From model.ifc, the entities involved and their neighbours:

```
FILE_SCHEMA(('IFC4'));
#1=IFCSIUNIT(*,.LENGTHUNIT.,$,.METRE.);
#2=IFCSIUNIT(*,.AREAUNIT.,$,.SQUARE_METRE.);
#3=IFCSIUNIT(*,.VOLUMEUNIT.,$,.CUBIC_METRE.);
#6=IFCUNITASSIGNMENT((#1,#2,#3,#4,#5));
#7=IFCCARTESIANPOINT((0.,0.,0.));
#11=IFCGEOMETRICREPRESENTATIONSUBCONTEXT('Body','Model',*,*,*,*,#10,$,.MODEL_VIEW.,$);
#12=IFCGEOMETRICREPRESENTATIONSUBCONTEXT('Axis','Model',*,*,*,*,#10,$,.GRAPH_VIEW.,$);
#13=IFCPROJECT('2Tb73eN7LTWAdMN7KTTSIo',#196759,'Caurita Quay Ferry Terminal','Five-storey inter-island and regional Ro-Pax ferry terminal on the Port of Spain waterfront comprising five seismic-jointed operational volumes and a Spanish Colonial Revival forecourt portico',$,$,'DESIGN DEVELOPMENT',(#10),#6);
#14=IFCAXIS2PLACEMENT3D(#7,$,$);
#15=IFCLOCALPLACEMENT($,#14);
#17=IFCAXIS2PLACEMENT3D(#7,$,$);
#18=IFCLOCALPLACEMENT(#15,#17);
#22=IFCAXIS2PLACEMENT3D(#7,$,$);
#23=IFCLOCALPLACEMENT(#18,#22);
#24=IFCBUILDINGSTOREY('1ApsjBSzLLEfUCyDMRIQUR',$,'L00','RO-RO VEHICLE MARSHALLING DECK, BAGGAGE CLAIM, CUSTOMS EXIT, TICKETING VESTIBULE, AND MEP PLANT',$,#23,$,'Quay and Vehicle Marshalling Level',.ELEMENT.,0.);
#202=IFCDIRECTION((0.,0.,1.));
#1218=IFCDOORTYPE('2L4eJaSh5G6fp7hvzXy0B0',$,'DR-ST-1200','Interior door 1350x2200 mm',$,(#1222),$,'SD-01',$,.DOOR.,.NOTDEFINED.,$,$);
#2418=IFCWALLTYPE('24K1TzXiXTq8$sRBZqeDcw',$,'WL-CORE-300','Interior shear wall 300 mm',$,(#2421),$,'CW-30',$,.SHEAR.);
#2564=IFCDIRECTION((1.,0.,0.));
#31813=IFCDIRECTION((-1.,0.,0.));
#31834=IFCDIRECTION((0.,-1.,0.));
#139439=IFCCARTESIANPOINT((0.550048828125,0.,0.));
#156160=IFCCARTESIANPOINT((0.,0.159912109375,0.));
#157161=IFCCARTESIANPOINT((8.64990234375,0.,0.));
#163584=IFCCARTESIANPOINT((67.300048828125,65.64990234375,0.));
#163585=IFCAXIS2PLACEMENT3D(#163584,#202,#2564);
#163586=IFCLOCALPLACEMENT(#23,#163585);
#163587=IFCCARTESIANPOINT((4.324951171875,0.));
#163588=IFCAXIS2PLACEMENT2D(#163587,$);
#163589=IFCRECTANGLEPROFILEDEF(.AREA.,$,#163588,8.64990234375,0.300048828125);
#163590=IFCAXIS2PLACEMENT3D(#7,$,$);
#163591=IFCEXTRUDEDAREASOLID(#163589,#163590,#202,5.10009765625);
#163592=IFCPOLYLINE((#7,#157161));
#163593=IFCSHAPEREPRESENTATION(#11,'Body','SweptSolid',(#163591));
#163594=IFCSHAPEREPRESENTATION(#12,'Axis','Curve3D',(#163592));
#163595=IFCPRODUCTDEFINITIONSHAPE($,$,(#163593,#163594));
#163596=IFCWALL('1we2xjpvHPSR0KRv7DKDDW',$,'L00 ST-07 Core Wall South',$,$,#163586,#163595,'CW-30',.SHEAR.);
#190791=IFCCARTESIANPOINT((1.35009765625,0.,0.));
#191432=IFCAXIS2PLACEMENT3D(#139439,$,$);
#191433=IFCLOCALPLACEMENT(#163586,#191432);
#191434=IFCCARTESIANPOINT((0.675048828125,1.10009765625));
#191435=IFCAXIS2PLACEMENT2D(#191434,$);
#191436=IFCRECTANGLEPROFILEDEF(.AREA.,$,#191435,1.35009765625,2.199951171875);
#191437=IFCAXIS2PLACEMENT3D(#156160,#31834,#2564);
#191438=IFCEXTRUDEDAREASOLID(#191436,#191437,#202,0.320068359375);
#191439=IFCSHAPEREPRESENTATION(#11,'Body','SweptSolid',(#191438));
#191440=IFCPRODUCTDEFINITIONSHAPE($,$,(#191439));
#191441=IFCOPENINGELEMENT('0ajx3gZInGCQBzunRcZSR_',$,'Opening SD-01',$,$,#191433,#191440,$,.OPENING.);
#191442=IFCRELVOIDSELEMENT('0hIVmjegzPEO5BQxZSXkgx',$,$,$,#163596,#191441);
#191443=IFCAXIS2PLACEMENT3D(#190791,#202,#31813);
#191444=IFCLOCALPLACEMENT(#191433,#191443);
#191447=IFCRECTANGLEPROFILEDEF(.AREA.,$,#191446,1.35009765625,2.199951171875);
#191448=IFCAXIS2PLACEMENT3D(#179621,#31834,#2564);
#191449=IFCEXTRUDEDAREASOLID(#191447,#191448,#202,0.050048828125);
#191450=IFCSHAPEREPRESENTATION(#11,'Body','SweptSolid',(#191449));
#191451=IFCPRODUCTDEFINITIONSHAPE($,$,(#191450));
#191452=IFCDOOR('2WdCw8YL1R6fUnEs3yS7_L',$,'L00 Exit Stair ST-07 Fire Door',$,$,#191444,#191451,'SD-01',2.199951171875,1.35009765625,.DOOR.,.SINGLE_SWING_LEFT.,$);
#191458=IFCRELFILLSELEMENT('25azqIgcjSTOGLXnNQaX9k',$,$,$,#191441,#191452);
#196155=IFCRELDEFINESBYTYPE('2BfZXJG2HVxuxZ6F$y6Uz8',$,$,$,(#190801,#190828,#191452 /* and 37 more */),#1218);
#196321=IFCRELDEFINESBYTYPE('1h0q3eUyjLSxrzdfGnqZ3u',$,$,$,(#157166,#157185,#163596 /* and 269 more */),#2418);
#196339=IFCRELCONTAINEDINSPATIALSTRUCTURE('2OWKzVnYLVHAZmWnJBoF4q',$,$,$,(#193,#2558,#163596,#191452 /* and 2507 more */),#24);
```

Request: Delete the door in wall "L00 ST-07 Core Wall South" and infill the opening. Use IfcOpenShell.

```python
import ifcopenshell
import ifcopenshell.api.feature
import ifcopenshell.api.root
import ifcopenshell.geom
import ifcopenshell.util.shape

model = ifcopenshell.open("model.ifc")
settings = ifcopenshell.geom.settings()


def volume(element):
    """Net volume in cubic metres, openings subtracted."""
    shape = ifcopenshell.geom.create_shape(settings, element)
    return ifcopenshell.util.shape.get_volume(shape.geometry)


door = model.by_guid("2WdCw8YL1R6fUnEs3yS7_L")
opening = door.FillsVoids[0].RelatingOpeningElement
wall = opening.VoidsElements[0].RelatingBuildingElement
before = volume(wall)

ifcopenshell.api.root.remove_product(model, product=door)
ifcopenshell.api.feature.remove_feature(model, feature=opening)

after = volume(wall)

print(f"wall volume {before:.3f} -> {after:.3f} m3")

model.write("model-out.ifc")
```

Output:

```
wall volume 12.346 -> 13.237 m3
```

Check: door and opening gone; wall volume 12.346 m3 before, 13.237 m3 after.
